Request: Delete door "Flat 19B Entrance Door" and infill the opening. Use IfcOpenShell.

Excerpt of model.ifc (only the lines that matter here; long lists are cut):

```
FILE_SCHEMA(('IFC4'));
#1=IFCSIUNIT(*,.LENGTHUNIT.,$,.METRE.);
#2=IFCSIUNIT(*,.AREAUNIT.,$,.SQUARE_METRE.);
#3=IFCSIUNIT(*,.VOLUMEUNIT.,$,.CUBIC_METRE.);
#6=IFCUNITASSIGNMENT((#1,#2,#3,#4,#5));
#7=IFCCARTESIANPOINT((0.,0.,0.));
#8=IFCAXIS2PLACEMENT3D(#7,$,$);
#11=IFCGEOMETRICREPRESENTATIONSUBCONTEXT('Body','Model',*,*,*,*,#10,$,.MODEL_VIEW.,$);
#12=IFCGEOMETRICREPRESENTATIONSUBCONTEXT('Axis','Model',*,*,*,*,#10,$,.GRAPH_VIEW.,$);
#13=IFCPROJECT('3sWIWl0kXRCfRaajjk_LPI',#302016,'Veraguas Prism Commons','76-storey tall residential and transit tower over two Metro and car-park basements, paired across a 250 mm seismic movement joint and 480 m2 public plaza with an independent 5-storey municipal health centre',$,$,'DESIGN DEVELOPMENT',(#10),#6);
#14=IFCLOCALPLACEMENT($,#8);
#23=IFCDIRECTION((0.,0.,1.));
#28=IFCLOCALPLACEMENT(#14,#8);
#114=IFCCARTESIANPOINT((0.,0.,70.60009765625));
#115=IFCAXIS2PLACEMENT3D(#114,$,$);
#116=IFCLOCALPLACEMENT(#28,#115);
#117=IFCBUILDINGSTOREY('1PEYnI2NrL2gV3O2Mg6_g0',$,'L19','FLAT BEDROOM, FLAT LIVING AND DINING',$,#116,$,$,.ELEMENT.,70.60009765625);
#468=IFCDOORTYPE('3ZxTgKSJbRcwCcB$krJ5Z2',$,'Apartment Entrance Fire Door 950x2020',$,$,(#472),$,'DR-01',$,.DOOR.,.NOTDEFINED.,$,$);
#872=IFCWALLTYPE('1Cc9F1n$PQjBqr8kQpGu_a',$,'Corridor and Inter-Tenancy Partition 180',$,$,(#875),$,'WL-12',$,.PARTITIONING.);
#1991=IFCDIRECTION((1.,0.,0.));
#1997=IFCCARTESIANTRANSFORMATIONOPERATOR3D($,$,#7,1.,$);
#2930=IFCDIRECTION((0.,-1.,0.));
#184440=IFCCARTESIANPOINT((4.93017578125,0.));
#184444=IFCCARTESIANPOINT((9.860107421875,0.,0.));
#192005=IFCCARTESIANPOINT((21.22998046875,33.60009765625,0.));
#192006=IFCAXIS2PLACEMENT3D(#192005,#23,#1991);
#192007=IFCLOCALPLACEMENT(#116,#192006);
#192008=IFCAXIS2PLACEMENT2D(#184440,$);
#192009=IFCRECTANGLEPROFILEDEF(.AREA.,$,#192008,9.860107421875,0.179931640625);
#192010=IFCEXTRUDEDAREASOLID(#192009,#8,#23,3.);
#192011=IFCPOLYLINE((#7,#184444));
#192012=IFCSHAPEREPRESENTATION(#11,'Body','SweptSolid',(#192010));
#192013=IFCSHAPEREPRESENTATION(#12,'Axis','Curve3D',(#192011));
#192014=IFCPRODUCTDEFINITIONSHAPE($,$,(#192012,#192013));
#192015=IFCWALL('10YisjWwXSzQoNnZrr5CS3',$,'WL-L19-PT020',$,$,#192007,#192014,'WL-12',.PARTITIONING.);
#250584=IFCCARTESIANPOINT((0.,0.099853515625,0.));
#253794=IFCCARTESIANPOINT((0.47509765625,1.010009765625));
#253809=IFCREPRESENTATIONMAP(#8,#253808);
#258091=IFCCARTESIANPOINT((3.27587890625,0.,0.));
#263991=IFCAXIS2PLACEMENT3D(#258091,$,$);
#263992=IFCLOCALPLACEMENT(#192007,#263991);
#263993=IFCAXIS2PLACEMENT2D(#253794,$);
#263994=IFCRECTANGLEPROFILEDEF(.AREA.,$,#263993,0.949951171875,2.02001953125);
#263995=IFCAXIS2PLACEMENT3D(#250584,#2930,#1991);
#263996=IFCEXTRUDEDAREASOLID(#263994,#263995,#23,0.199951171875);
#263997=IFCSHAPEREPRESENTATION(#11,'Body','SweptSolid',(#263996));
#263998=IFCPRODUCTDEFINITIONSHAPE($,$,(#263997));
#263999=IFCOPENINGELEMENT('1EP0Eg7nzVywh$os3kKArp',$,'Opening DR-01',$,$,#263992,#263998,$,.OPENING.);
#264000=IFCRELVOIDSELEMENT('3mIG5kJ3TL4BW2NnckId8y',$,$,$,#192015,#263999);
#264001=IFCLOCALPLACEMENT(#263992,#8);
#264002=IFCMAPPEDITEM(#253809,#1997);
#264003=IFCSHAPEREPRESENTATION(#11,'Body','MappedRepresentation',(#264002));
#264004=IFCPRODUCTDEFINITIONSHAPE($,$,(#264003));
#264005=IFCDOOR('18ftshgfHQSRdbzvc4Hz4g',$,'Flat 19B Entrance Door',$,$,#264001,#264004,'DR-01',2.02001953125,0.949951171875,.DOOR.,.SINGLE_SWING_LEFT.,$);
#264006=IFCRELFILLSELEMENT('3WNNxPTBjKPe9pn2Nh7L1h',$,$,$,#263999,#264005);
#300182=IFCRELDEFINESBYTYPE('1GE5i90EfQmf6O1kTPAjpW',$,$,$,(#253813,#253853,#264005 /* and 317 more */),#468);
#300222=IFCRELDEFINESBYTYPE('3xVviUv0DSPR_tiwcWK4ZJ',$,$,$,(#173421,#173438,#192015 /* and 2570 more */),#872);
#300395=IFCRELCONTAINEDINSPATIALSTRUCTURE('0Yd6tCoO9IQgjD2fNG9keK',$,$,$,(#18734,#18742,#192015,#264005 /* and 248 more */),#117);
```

```python
import ifcopenshell
import ifcopenshell.api.feature
import ifcopenshell.api.root
import ifcopenshell.geom
import ifcopenshell.util.shape

model = ifcopenshell.open("model.ifc")
settings = ifcopenshell.geom.settings()


def volume(element):
    """Net volume in cubic metres, openings subtracted."""
    shape = ifcopenshell.geom.create_shape(settings, element)
    return ifcopenshell.util.shape.get_volume(shape.geometry)


door = model.by_guid("18ftshgfHQSRdbzvc4Hz4g")
opening = door.FillsVoids[0].RelatingOpeningElement
wall = opening.VoidsElements[0].RelatingBuildingElement
before = volume(wall)

ifcopenshell.api.root.remove_product(model, product=door)
ifcopenshell.api.feature.remove_feature(model, feature=opening)

after = volume(wall)

print(f"wall volume {before:.3f} -> {after:.3f} m3")

model.write("model-out.ifc")
```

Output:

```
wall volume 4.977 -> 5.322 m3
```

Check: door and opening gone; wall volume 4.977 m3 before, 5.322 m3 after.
